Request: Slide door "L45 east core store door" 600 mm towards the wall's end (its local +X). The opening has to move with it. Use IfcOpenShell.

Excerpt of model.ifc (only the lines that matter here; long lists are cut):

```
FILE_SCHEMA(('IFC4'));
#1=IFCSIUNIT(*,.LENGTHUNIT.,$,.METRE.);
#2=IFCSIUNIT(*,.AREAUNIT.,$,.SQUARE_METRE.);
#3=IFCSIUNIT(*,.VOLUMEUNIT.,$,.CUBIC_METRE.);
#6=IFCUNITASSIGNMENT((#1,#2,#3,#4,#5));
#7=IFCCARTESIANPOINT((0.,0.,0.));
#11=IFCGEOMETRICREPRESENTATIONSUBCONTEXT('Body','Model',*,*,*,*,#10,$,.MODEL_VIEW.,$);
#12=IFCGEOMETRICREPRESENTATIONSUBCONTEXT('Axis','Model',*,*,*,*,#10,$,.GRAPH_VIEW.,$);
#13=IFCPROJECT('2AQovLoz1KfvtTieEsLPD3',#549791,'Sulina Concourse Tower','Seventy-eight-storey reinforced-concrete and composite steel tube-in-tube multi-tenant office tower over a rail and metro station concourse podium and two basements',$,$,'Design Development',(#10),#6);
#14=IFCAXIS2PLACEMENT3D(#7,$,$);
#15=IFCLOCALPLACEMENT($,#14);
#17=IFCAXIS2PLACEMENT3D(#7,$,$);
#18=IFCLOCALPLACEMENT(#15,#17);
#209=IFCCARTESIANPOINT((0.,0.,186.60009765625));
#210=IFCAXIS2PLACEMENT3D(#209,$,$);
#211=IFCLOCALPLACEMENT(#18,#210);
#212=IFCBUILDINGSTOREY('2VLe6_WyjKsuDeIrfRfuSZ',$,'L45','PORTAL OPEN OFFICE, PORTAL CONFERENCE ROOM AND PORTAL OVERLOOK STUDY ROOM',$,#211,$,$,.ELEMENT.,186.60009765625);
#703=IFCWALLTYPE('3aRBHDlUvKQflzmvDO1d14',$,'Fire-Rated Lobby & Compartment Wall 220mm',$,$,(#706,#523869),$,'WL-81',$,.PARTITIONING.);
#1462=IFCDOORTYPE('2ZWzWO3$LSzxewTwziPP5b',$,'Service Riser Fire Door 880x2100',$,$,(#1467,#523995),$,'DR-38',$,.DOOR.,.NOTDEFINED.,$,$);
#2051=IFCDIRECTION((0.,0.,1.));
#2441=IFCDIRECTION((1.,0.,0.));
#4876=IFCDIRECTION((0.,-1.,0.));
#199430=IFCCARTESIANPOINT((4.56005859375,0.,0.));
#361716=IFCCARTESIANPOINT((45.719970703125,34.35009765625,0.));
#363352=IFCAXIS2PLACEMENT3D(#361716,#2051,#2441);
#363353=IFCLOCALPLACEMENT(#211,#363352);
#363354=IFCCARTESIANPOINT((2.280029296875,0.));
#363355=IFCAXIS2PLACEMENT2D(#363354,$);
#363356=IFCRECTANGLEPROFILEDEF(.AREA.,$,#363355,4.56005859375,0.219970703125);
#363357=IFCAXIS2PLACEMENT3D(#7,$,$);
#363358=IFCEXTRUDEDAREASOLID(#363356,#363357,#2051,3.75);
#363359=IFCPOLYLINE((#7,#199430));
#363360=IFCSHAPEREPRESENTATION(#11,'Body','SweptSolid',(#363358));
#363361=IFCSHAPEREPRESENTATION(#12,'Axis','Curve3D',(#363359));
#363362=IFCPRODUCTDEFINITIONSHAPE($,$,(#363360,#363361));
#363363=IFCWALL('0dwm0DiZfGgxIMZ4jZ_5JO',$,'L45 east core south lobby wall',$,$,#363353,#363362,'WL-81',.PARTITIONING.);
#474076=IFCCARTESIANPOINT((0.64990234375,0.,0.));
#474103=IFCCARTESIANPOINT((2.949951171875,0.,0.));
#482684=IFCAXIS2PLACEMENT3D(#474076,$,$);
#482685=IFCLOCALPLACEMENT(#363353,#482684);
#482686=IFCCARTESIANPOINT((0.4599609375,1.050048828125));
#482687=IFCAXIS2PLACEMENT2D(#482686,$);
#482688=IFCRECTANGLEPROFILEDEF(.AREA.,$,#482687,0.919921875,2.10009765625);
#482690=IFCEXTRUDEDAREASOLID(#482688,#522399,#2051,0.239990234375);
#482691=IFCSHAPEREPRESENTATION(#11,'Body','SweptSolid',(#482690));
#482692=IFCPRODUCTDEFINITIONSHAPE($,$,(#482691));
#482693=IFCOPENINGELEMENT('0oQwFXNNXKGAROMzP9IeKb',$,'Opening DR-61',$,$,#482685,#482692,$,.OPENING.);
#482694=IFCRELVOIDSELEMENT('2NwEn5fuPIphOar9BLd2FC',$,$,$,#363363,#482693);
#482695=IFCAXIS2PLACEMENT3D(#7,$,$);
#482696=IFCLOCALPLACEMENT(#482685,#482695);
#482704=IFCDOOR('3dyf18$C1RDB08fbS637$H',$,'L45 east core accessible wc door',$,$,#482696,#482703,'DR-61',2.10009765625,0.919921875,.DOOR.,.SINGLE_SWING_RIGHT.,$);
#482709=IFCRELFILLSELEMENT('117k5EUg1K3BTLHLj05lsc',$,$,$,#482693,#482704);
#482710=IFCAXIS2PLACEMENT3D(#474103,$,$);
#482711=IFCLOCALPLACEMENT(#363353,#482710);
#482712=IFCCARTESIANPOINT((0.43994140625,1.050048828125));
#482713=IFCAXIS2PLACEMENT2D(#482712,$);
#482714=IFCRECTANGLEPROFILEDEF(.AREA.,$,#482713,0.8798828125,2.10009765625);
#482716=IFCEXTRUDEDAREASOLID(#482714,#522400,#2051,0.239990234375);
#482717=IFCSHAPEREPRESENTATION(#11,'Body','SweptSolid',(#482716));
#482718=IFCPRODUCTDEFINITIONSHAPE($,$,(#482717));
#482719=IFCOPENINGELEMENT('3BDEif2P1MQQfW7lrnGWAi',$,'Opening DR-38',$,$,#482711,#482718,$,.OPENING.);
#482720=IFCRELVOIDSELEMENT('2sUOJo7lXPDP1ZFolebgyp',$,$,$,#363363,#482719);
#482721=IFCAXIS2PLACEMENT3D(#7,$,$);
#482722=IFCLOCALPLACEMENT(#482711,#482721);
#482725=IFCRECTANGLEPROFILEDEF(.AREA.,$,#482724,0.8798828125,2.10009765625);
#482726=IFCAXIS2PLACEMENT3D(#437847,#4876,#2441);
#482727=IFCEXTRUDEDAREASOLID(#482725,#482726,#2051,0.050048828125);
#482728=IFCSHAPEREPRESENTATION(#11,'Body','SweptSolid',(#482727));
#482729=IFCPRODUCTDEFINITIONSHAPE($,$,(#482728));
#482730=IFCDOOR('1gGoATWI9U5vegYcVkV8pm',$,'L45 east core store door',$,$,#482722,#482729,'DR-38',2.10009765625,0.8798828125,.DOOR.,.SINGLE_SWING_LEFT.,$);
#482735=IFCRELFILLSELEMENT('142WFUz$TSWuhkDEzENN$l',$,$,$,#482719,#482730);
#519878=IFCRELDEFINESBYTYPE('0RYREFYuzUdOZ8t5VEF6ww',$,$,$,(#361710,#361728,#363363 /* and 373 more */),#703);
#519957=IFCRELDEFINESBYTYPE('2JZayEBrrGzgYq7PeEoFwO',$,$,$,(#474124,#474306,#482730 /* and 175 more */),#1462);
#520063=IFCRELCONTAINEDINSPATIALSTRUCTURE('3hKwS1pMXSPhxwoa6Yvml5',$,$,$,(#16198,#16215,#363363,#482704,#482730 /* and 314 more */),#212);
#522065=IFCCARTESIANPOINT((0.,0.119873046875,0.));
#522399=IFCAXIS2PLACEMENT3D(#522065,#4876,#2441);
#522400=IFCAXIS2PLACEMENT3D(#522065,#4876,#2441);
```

```python
import ifcopenshell
import ifcopenshell.api.geometry
import ifcopenshell.util.placement

model = ifcopenshell.open("model.ifc")

door = model.by_id(482730)
opening = door.FillsVoids[0].RelatingOpeningElement
wall = opening.VoidsElements[0].RelatingBuildingElement

wall_matrix = ifcopenshell.util.placement.get_local_placement(wall.ObjectPlacement)
shift = wall_matrix[:3, 0] * 0.6
before = ifcopenshell.util.placement.get_local_placement(door.ObjectPlacement)[:3, 3].copy()

# The door is placed relative to its opening, so it follows when the opening moves.
matrix = ifcopenshell.util.placement.get_local_placement(opening.ObjectPlacement)
matrix[:3, 3] += shift
ifcopenshell.api.geometry.edit_object_placement(
    model, product=opening, matrix=matrix, is_si=False, should_transform_children=True
)

after = ifcopenshell.util.placement.get_local_placement(door.ObjectPlacement)[:3, 3]
print("door moved by", (after - before).round(3) + 0.0)

model.write("model-out.ifc")
```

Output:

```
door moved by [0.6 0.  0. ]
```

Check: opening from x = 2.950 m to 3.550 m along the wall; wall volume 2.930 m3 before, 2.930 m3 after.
